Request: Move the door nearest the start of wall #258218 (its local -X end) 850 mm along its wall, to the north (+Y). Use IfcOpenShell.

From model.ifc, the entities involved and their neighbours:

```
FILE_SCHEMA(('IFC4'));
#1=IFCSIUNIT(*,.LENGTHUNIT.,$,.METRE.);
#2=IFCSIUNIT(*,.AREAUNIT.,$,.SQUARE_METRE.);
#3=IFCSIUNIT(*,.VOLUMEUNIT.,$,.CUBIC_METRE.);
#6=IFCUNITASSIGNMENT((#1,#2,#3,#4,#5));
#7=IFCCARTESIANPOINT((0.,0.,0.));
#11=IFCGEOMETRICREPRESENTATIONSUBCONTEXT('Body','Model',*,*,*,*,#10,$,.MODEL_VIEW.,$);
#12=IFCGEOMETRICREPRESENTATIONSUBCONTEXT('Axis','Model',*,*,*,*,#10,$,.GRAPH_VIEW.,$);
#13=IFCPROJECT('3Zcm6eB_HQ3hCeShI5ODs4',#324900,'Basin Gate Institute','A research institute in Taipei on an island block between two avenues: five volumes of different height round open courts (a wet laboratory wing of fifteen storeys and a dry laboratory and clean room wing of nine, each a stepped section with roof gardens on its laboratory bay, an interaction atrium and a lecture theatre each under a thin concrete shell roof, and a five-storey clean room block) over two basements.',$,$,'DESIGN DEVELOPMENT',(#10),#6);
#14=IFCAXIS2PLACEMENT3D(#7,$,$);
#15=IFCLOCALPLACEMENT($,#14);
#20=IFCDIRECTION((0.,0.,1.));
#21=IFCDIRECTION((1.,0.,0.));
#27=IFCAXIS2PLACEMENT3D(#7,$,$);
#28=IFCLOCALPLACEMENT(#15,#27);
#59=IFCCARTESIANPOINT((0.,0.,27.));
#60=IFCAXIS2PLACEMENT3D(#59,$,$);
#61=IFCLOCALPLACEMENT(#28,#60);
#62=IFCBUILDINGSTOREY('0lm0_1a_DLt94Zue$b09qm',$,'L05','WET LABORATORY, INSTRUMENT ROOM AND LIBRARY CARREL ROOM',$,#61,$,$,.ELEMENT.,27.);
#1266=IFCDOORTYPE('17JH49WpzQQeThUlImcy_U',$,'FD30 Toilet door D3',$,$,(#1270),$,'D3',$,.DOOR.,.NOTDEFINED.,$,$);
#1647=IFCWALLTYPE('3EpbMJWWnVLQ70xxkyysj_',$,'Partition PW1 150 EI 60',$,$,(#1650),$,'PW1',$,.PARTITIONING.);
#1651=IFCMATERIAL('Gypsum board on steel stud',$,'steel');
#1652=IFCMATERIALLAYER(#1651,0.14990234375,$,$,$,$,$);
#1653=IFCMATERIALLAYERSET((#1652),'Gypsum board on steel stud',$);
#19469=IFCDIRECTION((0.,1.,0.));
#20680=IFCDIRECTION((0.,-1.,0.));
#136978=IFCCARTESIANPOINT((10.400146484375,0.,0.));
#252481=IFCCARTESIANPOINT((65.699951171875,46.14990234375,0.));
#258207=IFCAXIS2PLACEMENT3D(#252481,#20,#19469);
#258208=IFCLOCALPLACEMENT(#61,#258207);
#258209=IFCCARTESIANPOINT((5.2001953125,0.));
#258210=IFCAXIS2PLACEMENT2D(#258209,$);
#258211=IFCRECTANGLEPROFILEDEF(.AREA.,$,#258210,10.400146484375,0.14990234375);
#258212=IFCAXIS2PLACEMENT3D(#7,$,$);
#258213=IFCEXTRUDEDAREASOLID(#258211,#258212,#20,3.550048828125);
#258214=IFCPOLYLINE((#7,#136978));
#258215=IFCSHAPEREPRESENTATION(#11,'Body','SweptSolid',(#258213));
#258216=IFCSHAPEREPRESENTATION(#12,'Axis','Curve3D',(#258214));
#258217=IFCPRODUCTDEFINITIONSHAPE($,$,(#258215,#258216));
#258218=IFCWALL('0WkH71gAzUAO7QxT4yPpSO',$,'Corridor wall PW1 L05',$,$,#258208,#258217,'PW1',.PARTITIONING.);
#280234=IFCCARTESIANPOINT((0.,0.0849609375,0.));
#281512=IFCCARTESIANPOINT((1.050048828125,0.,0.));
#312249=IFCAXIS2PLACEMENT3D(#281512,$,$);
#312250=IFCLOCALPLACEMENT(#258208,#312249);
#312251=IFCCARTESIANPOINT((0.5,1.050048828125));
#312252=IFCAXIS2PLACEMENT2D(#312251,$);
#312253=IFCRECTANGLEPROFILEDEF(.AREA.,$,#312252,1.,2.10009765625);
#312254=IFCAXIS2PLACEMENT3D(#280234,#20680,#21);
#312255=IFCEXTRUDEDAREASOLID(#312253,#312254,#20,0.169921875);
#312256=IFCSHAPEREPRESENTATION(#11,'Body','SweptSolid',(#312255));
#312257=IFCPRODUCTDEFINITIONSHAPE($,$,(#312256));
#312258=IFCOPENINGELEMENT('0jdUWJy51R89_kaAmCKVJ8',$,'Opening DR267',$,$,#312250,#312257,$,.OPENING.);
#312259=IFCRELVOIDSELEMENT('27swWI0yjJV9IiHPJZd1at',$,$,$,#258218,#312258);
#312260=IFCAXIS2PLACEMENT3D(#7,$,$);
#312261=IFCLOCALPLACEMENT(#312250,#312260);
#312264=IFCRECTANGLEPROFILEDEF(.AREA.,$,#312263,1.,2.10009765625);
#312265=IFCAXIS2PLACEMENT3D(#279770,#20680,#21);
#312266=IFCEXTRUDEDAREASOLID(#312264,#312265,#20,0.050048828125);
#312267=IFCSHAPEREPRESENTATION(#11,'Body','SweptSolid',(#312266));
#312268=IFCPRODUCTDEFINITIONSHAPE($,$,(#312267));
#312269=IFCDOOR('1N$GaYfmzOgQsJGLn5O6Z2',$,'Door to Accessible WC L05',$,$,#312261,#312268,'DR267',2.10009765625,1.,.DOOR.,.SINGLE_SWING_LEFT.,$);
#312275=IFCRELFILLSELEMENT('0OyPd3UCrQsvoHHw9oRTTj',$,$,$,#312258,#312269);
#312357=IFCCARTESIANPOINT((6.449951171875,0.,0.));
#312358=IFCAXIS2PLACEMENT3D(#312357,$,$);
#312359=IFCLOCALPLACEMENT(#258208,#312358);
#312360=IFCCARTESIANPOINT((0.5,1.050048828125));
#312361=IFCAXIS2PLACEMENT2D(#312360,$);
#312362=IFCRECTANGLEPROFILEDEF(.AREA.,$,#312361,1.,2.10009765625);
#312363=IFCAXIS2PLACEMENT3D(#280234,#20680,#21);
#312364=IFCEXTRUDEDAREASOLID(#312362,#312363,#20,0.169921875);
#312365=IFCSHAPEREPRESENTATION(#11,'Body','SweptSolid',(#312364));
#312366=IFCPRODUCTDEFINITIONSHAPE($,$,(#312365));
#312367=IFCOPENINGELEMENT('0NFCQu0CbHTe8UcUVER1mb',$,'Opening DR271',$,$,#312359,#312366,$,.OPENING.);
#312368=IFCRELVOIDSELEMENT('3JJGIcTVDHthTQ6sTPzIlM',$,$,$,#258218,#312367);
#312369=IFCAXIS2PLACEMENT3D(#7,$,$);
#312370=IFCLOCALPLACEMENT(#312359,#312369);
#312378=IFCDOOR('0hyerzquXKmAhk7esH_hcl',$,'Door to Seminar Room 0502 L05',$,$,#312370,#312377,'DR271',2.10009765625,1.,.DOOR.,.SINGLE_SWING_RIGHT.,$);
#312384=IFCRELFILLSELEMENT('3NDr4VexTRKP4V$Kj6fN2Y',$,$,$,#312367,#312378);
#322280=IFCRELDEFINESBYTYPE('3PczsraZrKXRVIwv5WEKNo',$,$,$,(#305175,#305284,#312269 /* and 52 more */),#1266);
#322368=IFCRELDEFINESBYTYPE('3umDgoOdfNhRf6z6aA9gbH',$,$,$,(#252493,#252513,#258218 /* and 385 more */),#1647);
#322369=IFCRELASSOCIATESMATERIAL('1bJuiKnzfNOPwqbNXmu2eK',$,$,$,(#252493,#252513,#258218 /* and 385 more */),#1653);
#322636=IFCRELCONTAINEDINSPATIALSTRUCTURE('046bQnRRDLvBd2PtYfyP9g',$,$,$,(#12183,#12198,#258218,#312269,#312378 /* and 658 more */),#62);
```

```python
import ifcopenshell
import ifcopenshell.api.geometry
import ifcopenshell.util.placement

model = ifcopenshell.open("model.ifc")

door = model.by_guid("1N$GaYfmzOgQsJGLn5O6Z2")
opening = door.FillsVoids[0].RelatingOpeningElement
wall = opening.VoidsElements[0].RelatingBuildingElement

wall_matrix = ifcopenshell.util.placement.get_local_placement(wall.ObjectPlacement)
shift = wall_matrix[:3, 0] * 0.85
before = ifcopenshell.util.placement.get_local_placement(door.ObjectPlacement)[:3, 3].copy()

# The door is placed relative to its opening, so it follows when the opening moves.
matrix = ifcopenshell.util.placement.get_local_placement(opening.ObjectPlacement)
matrix[:3, 3] += shift
ifcopenshell.api.geometry.edit_object_placement(
    model, product=opening, matrix=matrix, is_si=False, should_transform_children=True
)

after = ifcopenshell.util.placement.get_local_placement(door.ObjectPlacement)[:3, 3]
print("door moved by", (after - before).round(3) + 0.0)

model.write("model_updated.ifc")
```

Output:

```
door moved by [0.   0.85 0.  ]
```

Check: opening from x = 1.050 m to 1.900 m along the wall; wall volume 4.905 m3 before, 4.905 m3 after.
